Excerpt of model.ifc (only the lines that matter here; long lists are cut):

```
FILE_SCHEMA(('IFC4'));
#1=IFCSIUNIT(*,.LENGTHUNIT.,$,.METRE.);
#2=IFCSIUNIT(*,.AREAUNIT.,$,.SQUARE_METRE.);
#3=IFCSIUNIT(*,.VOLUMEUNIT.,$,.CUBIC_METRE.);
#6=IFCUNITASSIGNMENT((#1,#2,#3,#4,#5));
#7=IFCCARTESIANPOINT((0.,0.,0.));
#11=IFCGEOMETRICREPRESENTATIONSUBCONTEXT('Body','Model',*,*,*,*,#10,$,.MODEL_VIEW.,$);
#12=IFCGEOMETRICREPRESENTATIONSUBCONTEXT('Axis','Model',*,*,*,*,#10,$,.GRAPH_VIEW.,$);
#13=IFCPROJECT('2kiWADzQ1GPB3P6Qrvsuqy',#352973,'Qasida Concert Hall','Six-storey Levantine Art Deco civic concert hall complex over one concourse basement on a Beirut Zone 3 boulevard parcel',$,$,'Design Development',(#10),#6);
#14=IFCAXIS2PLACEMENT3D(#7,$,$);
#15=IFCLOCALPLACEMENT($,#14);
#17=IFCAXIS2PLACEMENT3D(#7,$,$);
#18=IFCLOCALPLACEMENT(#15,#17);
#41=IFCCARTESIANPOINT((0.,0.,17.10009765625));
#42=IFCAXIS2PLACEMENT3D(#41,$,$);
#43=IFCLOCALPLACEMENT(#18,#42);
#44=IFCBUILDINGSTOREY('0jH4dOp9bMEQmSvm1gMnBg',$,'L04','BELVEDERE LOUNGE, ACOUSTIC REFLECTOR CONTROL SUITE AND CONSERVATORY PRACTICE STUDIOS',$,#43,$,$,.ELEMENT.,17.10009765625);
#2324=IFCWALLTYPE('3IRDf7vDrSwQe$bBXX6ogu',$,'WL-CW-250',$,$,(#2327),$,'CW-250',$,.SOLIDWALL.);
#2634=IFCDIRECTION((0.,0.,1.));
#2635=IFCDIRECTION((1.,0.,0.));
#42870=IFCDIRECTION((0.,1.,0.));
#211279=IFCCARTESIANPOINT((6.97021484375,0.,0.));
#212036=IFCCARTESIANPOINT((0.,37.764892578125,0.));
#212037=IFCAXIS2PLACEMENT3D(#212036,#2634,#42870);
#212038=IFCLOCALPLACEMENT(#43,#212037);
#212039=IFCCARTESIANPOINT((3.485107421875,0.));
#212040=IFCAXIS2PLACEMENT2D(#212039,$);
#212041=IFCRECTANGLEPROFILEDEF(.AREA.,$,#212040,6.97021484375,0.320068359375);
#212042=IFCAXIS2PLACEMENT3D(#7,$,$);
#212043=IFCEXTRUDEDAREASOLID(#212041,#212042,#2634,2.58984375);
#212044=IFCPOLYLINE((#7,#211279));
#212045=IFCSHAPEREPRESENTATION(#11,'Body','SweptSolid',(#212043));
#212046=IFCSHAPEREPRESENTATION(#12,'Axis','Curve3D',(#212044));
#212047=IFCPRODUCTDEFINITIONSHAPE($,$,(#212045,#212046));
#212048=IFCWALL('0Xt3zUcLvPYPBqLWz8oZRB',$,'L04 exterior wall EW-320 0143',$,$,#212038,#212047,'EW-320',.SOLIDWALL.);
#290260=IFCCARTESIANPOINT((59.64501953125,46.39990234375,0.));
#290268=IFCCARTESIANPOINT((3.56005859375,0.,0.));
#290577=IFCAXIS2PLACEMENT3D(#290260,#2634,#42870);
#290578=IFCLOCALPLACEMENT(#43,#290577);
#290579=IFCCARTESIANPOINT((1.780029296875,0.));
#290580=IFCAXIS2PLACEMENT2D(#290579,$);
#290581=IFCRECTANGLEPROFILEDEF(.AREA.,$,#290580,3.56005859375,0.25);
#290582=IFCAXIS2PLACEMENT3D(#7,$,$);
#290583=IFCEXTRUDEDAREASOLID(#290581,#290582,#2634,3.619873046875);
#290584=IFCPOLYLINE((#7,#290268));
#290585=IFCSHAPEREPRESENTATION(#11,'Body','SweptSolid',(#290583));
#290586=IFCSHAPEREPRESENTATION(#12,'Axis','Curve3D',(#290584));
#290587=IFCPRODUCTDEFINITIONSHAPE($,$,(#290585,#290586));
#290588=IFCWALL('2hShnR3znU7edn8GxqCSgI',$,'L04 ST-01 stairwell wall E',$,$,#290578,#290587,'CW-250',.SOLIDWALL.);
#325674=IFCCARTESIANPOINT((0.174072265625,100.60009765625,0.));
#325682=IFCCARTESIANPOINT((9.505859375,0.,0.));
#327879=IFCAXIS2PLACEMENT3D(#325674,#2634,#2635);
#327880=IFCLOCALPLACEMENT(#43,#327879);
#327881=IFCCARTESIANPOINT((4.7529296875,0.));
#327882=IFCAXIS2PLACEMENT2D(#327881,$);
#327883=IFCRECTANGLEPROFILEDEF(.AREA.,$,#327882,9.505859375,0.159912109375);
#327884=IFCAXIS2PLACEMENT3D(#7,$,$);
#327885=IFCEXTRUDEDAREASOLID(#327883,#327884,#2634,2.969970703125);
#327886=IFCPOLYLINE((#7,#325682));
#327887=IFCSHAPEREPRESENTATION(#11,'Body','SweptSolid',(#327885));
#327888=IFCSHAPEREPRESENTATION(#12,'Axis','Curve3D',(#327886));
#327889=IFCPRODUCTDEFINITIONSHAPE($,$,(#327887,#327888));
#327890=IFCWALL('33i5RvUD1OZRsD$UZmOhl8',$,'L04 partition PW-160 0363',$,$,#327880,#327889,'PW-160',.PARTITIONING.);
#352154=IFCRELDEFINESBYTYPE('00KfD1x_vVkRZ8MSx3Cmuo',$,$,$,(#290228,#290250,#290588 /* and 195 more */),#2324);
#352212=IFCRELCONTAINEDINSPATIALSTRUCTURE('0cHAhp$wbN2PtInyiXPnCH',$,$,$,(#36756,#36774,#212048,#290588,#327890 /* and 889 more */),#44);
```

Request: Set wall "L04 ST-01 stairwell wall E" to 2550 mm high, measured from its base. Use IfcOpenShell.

```python
import ifcopenshell
import ifcopenshell.geom
import ifcopenshell.util.representation
import ifcopenshell.util.shape
import ifcopenshell.util.unit

model = ifcopenshell.open("model.ifc")
unit_scale = ifcopenshell.util.unit.calculate_unit_scale(model)
settings = ifcopenshell.geom.settings()


def volume(element):
    """Net volume in cubic metres, openings subtracted."""
    shape = ifcopenshell.geom.create_shape(settings, element)
    return ifcopenshell.util.shape.get_volume(shape.geometry)


wall = model.by_guid("2hShnR3znU7edn8GxqCSgI")
before = volume(wall)

body = ifcopenshell.util.representation.get_representation(wall, "Model", "Body")
solid = body.Items[0]
old_height = solid.Depth
solid.Depth = 2.55 / unit_scale
after = volume(wall)

print(f"height {old_height:g} -> {solid.Depth:g}, volume {before:.3f} -> {after:.3f} m3")

model.write("model-out.ifc")
```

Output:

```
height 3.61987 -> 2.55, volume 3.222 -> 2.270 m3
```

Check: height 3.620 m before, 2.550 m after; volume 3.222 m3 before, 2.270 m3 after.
